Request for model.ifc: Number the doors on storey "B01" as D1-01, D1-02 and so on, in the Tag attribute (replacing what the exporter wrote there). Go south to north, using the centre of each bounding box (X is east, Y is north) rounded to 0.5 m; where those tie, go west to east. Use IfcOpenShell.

First a look at what the model holds.

```python
import ifcopenshell
import ifcopenshell.util.element
import ifcopenshell.util.placement

model = ifcopenshell.open("model.ifc")
print(model.schema)
storey = next(s for s in model.by_type("IfcBuildingStorey") if s.Name == "B01")
doors = [e for e in ifcopenshell.util.element.get_decomposition(storey) if e.is_a("IfcDoor")]
for e in sorted(doors, key=lambda e: e.id()):
    origin = ifcopenshell.util.placement.get_local_placement(e.ObjectPlacement)[:3, 3]
    print(e.id(), e.Tag, e.Name, origin.round(2) + 0.0, sep=" | ")
```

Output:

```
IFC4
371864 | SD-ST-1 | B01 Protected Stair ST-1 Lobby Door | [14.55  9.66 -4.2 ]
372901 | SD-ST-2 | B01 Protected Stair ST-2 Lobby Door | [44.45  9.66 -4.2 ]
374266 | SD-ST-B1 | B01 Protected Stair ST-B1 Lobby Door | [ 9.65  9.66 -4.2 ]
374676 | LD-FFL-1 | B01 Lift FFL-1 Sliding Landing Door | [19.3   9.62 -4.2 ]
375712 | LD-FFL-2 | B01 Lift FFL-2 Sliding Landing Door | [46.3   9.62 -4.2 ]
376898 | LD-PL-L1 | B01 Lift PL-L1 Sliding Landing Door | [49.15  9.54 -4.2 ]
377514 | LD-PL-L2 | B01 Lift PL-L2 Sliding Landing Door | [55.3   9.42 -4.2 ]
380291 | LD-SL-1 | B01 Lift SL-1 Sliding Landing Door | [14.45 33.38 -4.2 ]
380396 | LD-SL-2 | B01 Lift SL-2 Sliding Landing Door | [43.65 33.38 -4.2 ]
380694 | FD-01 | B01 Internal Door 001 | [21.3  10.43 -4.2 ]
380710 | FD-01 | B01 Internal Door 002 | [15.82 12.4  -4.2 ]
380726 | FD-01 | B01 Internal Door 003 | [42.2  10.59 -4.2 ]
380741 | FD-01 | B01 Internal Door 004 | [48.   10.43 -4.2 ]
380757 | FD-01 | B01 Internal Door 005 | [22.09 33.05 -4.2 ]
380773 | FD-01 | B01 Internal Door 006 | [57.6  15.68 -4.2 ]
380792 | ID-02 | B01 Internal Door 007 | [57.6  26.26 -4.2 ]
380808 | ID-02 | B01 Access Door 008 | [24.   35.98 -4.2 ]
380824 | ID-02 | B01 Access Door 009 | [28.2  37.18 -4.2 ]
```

```python
import ifcopenshell
import ifcopenshell.geom
import ifcopenshell.util.element
import ifcopenshell.util.shape

model = ifcopenshell.open("model.ifc")
settings = ifcopenshell.geom.settings()
settings.set("use-world-coords", True)


def centre(element):
    shape = ifcopenshell.geom.create_shape(settings, element)
    return ifcopenshell.util.shape.get_bbox_centroid(shape.geometry)


storey = next(s for s in model.by_type("IfcBuildingStorey") if s.Name == "B01")
doors = [e for e in ifcopenshell.util.element.get_decomposition(storey) if e.is_a("IfcDoor")]

# Insertion points can sit at a corner or the storey origin, so sort by the geometry (in metres).
centres = {e: centre(e) for e in doors}
doors.sort(key=lambda e: (round(centres[e][1] / 0.5), centres[e][0]))

for i, e in enumerate(doors, start=1):
    number = f"D1-{i:02d}"
    e.Tag = number
    print(e.id(), number)

model.write("model_v2.ifc")
```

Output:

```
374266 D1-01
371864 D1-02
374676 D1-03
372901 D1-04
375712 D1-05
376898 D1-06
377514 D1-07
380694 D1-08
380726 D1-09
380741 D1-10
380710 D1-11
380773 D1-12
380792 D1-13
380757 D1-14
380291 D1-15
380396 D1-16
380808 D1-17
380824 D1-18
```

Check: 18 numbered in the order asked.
